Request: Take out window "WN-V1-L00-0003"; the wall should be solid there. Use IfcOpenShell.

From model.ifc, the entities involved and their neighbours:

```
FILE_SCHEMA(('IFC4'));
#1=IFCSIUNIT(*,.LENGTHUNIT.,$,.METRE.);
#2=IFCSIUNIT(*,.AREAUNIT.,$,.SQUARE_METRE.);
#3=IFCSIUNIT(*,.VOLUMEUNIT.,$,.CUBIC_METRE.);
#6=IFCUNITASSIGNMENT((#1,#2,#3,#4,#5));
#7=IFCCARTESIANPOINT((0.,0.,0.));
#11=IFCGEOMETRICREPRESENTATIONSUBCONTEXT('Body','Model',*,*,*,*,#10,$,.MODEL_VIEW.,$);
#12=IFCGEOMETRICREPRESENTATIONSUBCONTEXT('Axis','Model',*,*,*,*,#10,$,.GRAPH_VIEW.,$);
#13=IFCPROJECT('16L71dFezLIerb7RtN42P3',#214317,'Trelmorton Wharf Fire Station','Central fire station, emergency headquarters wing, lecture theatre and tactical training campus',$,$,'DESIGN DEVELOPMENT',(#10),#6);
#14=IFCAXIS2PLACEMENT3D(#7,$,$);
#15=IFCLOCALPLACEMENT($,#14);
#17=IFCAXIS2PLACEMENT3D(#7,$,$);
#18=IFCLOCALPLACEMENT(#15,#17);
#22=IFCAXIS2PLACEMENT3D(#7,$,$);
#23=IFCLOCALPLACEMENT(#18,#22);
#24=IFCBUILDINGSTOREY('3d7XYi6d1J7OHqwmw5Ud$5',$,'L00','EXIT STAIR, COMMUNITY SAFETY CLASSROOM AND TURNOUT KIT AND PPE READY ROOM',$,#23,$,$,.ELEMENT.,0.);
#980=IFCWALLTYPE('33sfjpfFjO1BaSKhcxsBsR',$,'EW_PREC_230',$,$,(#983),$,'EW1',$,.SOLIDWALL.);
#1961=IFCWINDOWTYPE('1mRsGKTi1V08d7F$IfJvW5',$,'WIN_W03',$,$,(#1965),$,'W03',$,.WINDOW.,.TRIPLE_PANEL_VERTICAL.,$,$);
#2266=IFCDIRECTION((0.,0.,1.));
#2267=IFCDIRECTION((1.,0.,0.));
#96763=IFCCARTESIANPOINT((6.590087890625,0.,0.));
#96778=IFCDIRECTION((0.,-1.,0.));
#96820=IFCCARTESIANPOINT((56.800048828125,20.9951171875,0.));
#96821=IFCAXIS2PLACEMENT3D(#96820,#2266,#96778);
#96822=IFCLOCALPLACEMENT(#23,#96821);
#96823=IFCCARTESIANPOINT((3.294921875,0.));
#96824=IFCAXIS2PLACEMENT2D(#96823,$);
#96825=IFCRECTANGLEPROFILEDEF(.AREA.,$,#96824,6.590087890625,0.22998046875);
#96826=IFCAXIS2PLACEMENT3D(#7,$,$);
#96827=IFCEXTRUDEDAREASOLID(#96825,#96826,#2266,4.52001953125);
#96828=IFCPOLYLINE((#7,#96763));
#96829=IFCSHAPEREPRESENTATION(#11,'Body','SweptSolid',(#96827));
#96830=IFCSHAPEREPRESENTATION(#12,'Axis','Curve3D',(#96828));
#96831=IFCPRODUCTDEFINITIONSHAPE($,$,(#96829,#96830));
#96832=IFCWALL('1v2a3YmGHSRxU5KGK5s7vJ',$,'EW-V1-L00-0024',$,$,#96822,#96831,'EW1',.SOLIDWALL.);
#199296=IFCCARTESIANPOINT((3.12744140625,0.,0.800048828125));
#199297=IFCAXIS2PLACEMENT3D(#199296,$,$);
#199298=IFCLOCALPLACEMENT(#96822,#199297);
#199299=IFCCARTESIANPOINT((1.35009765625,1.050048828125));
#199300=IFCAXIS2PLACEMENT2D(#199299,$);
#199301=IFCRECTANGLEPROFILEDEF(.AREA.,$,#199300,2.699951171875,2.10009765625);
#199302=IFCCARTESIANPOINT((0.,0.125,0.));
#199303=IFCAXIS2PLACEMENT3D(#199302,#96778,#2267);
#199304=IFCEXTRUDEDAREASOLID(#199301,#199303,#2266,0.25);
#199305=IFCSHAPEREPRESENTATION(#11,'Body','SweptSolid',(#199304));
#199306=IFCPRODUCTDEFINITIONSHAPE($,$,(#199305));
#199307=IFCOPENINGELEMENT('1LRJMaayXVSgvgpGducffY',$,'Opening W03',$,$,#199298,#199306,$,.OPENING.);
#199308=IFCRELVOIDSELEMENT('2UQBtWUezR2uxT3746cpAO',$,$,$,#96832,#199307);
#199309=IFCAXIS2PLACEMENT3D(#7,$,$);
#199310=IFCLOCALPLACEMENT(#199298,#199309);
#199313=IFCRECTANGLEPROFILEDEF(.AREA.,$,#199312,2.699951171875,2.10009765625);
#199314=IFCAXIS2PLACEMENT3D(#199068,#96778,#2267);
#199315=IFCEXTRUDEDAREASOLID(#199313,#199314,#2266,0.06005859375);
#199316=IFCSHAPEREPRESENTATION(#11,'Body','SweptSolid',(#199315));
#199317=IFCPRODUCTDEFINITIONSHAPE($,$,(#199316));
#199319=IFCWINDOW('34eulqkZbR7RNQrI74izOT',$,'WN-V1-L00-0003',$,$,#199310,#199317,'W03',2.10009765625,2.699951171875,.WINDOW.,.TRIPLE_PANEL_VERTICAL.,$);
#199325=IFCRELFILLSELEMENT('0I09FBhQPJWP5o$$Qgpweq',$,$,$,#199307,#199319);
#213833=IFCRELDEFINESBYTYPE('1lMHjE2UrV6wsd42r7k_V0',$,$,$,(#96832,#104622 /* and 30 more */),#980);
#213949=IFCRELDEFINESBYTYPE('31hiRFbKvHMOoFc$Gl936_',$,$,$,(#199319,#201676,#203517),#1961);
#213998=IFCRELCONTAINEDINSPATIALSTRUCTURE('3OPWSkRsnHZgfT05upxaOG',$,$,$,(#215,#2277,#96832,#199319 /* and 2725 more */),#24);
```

```python
import ifcopenshell
import ifcopenshell.api.feature
import ifcopenshell.api.root
import ifcopenshell.geom
import ifcopenshell.util.shape

model = ifcopenshell.open("model.ifc")
settings = ifcopenshell.geom.settings()


def volume(element):
    """Net volume in cubic metres, openings subtracted."""
    shape = ifcopenshell.geom.create_shape(settings, element)
    return ifcopenshell.util.shape.get_volume(shape.geometry)


window = model.by_id(199319)
opening = window.FillsVoids[0].RelatingOpeningElement
wall = opening.VoidsElements[0].RelatingBuildingElement
before = volume(wall)

ifcopenshell.api.root.remove_product(model, product=window)
ifcopenshell.api.feature.remove_feature(model, feature=opening)

after = volume(wall)

print(f"wall volume {before:.3f} -> {after:.3f} m3")

model.write("model-out.ifc")
```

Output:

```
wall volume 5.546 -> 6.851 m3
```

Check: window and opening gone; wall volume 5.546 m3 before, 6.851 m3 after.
